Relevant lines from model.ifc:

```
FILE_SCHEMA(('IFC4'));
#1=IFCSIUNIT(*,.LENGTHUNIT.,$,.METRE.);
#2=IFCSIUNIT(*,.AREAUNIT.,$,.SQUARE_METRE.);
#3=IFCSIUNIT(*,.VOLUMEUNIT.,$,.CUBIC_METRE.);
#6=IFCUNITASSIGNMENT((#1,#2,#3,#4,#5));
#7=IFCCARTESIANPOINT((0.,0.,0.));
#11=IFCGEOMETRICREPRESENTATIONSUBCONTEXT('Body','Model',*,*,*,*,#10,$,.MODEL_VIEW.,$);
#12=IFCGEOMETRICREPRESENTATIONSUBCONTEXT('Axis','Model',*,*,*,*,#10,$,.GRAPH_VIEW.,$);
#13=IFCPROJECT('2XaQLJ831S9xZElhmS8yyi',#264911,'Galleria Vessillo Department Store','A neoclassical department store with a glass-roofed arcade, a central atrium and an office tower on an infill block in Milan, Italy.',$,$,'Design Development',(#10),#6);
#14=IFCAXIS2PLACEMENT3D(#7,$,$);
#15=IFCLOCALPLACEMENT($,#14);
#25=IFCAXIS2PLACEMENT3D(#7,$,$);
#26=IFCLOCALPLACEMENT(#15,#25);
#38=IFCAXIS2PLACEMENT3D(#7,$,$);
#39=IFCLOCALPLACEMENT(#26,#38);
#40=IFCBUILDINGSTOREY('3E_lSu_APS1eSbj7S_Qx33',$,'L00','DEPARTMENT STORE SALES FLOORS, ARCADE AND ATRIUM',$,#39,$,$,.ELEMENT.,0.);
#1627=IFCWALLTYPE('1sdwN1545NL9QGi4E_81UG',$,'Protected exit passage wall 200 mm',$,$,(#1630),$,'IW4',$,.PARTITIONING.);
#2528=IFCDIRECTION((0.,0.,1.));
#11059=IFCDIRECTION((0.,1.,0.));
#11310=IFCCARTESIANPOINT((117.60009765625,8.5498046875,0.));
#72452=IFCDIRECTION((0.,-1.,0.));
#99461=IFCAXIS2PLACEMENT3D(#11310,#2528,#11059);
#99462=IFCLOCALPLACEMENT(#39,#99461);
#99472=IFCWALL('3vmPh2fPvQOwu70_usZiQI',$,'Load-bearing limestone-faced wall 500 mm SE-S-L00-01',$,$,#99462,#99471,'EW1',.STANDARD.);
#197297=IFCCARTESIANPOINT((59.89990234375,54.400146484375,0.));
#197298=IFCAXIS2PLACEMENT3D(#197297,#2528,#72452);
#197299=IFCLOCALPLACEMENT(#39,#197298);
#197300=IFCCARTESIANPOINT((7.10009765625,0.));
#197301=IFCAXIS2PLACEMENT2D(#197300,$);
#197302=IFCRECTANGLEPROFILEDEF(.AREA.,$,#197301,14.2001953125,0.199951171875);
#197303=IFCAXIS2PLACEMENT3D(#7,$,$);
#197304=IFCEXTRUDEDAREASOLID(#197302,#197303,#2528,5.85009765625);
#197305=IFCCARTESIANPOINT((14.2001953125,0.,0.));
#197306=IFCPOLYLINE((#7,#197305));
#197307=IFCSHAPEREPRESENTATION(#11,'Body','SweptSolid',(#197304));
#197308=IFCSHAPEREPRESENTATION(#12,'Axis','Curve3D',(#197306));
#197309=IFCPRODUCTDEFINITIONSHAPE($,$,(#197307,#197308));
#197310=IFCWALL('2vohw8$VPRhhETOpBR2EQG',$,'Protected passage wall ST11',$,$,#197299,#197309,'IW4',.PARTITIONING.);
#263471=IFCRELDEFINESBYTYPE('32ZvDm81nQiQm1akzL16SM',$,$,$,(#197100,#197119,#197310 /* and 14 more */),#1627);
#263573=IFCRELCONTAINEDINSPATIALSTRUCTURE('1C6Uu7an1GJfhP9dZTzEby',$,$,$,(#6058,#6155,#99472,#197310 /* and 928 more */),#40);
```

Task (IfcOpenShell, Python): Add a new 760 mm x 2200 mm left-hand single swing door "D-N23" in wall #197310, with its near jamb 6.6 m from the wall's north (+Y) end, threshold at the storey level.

```python
import numpy as np
import ifcopenshell
import ifcopenshell.api.feature
import ifcopenshell.api.geometry
import ifcopenshell.api.root
import ifcopenshell.api.spatial
import ifcopenshell.geom
import ifcopenshell.util.element
import ifcopenshell.util.placement
import ifcopenshell.util.representation
import ifcopenshell.util.shape
import ifcopenshell.util.unit

model = ifcopenshell.open("model.ifc")
unit_scale = ifcopenshell.util.unit.calculate_unit_scale(model)
settings = ifcopenshell.geom.settings()


def volume(element):
    """Net volume in cubic metres, openings subtracted."""
    shape = ifcopenshell.geom.create_shape(settings, element)
    return ifcopenshell.util.shape.get_volume(shape.geometry)


wall = model.by_id(197310)
storey = ifcopenshell.util.element.get_container(wall, ifc_class="IfcBuildingStorey")
context = ifcopenshell.util.representation.get_context(model, "Model", "Body", "MODEL_VIEW")
before = volume(wall)

width, height, from_end, sill = 0.76, 2.2, 6.6, 0.0  # metres

# The wall runs along its own X axis, and the end named is its -X end.
wall_shape = ifcopenshell.geom.create_shape(settings, wall)
x, y, z = ifcopenshell.util.shape.get_vertices(wall_shape.geometry).T
start = x.min() + from_end
face, thickness = float(y.min()), float(y.max() - y.min())
wall_matrix = ifcopenshell.util.placement.get_local_placement(wall.ObjectPlacement)
level = ifcopenshell.util.placement.get_local_placement(storey.ObjectPlacement)[2, 3]


def in_wall(x, y):
    """Placement at x, y metres in the wall's axes, at sill height."""
    matrix = wall_matrix.copy()
    matrix[:, 3] = wall_matrix @ np.array([x / unit_scale, y / unit_scale, 0.0, 1.0])
    matrix[2, 3] = level + sill / unit_scale
    return matrix


# Opening: a box that overshoots both wall faces by 50 mm.
opening = ifcopenshell.api.root.create_entity(model, ifc_class="IfcOpeningElement", predefined_type="OPENING")
box = ifcopenshell.api.geometry.add_wall_representation(
    model, context=context, length=width, height=height, thickness=thickness + 0.1
)
ifcopenshell.api.geometry.assign_representation(model, product=opening, representation=box)
ifcopenshell.api.geometry.edit_object_placement(model, product=opening, matrix=in_wall(start, face - 0.05), is_si=False)
ifcopenshell.api.feature.add_feature(model, feature=opening, element=wall)

door = ifcopenshell.api.root.create_entity(model, ifc_class="IfcDoor", name="D-N23", predefined_type="DOOR")
door.OverallWidth, door.OverallHeight = width / unit_scale, height / unit_scale
door.OperationType = "SINGLE_SWING_LEFT"
body = ifcopenshell.api.geometry.add_door_representation(
    model,
    context=context,
    overall_width=door.OverallWidth,
    overall_height=door.OverallHeight,
    operation_type="SINGLE_SWING_LEFT",
    lining_properties={"LiningDepth": thickness / unit_scale, "ThresholdDepth": thickness / unit_scale},
)
ifcopenshell.api.geometry.assign_representation(model, product=door, representation=body)
ifcopenshell.api.spatial.assign_container(model, products=[door], relating_structure=storey)
ifcopenshell.api.feature.add_filling(model, opening=opening, element=door)

# The lining spans the wall, so the door starts at the wall face.
ifcopenshell.api.geometry.edit_object_placement(model, product=door, matrix=in_wall(start, face), is_si=False)

after = volume(wall)

print(f"wall volume {before:.3f} -> {after:.3f} m3")

model.write("model-out.ifc")
```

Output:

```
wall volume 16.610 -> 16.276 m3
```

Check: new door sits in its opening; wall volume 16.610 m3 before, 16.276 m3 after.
